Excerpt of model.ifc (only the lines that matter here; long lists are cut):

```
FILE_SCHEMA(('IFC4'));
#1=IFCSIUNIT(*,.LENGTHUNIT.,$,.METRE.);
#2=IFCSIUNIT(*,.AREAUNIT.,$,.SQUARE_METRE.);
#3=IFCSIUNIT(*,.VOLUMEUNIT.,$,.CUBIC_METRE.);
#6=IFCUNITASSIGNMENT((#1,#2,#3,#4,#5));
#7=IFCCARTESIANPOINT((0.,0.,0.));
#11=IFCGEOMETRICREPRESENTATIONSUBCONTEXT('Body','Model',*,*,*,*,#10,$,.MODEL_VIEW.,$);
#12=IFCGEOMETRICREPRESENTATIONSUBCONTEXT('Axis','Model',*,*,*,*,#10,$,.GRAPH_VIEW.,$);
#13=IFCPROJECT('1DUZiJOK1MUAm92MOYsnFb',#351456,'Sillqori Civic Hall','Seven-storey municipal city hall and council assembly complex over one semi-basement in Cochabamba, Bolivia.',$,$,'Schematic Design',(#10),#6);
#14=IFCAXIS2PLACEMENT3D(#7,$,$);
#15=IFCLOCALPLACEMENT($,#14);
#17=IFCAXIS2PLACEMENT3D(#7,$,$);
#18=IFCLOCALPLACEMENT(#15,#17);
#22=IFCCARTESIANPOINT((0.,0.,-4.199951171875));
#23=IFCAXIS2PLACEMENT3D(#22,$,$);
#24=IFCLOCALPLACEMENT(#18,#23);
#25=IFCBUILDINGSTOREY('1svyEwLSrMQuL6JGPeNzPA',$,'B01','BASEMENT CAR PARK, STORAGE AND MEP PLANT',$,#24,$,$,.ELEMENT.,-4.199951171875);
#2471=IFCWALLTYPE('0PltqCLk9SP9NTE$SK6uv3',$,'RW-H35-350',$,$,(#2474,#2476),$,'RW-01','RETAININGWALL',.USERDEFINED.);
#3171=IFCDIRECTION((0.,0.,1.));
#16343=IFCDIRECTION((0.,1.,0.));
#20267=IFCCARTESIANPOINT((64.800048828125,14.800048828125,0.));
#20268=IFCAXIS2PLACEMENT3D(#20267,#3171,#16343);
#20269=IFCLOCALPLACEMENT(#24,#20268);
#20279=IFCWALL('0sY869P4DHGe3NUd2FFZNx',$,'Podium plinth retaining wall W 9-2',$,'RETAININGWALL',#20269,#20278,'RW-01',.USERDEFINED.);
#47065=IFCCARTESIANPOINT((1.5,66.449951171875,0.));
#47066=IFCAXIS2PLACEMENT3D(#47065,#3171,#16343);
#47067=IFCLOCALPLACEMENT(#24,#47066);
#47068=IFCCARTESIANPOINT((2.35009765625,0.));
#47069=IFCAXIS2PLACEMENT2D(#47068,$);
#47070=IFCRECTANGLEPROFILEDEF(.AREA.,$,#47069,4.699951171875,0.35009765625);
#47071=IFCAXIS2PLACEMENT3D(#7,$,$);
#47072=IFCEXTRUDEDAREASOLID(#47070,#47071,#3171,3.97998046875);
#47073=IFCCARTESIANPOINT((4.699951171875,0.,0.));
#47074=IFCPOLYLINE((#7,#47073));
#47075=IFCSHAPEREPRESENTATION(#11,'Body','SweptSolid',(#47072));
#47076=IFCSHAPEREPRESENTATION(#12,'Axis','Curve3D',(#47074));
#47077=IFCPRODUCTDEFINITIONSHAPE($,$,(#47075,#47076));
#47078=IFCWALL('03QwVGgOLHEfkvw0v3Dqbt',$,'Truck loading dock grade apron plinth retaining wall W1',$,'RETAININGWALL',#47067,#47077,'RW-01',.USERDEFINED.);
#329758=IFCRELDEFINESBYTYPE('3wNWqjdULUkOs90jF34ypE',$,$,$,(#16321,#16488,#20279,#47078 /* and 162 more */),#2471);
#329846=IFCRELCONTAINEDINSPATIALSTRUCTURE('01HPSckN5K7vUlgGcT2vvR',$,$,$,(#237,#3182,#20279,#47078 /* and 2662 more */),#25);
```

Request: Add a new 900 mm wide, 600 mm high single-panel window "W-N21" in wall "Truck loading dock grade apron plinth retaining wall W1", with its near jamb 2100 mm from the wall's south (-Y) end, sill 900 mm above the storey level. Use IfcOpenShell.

```python
import numpy as np
import ifcopenshell
import ifcopenshell.api.feature
import ifcopenshell.api.geometry
import ifcopenshell.api.root
import ifcopenshell.api.spatial
import ifcopenshell.geom
import ifcopenshell.util.element
import ifcopenshell.util.placement
import ifcopenshell.util.representation
import ifcopenshell.util.shape
import ifcopenshell.util.unit

model = ifcopenshell.open("model.ifc")
unit_scale = ifcopenshell.util.unit.calculate_unit_scale(model)
settings = ifcopenshell.geom.settings()


def volume(element):
    """Net volume in cubic metres, openings subtracted."""
    shape = ifcopenshell.geom.create_shape(settings, element)
    return ifcopenshell.util.shape.get_volume(shape.geometry)


wall = model.by_id(47078)
storey = ifcopenshell.util.element.get_container(wall, ifc_class="IfcBuildingStorey")
context = ifcopenshell.util.representation.get_context(model, "Model", "Body", "MODEL_VIEW")
before = volume(wall)

width, height, from_end, sill = 0.9, 0.6, 2.1, 0.9  # metres

# The wall runs along its own X axis, and the end named is its -X end.
wall_shape = ifcopenshell.geom.create_shape(settings, wall)
x, y, z = ifcopenshell.util.shape.get_vertices(wall_shape.geometry).T
start = x.min() + from_end
face, thickness = float(y.min()), float(y.max() - y.min())
wall_matrix = ifcopenshell.util.placement.get_local_placement(wall.ObjectPlacement)
level = ifcopenshell.util.placement.get_local_placement(storey.ObjectPlacement)[2, 3]


def in_wall(x, y):
    """Placement at x, y metres in the wall's axes, at sill height."""
    matrix = wall_matrix.copy()
    matrix[:, 3] = wall_matrix @ np.array([x / unit_scale, y / unit_scale, 0.0, 1.0])
    matrix[2, 3] = level + sill / unit_scale
    return matrix


# Opening: a box that overshoots both wall faces by 50 mm.
opening = ifcopenshell.api.root.create_entity(model, ifc_class="IfcOpeningElement", predefined_type="OPENING")
box = ifcopenshell.api.geometry.add_wall_representation(
    model, context=context, length=width, height=height, thickness=thickness + 0.1
)
ifcopenshell.api.geometry.assign_representation(model, product=opening, representation=box)
ifcopenshell.api.geometry.edit_object_placement(model, product=opening, matrix=in_wall(start, face - 0.05), is_si=False)
ifcopenshell.api.feature.add_feature(model, feature=opening, element=wall)

window = ifcopenshell.api.root.create_entity(model, ifc_class="IfcWindow", name="W-N21", predefined_type="WINDOW")
window.OverallWidth, window.OverallHeight = width / unit_scale, height / unit_scale
window.PartitioningType = "SINGLE_PANEL"
body = ifcopenshell.api.geometry.add_window_representation(
    model,
    context=context,
    overall_width=window.OverallWidth,
    overall_height=window.OverallHeight,
    partition_type="SINGLE_PANEL",
)
ifcopenshell.api.geometry.assign_representation(model, product=window, representation=body)
ifcopenshell.api.spatial.assign_container(model, products=[window], relating_structure=storey)
ifcopenshell.api.feature.add_filling(model, opening=opening, element=window)

# Centre the window in the wall's thickness.
ifcopenshell.api.geometry.edit_object_placement(model, product=window, matrix=in_wall(start, face), is_si=False)
window_shape = ifcopenshell.geom.create_shape(settings, window)
depth = ifcopenshell.util.shape.get_vertices(window_shape.geometry)[:, 1]
offset = face + thickness / 2 - (depth.min() + depth.max()) / 2
ifcopenshell.api.geometry.edit_object_placement(model, product=window, matrix=in_wall(start, offset), is_si=False)

after = volume(wall)

print(f"wall volume {before:.3f} -> {after:.3f} m3")

model.write("model_updated.ifc")
```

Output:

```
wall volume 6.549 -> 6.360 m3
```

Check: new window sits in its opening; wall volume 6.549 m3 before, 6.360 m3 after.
